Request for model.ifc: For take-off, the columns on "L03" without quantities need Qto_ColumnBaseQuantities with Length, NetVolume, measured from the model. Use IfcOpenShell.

First a look at what the model holds.

```python
import ifcopenshell
import ifcopenshell.util.element
import ifcopenshell.util.unit

model = ifcopenshell.open("model.ifc")
print(model.schema)
for unit_type in ("LENGTHUNIT", "AREAUNIT", "VOLUMEUNIT"):
    print(unit_type, ifcopenshell.util.unit.calculate_unit_scale(model, unit_type))
storey = next(s for s in model.by_type("IfcBuildingStorey") if s.Name == "L03")
columns = [e for e in ifcopenshell.util.element.get_decomposition(storey) if e.is_a("IfcColumn")]
for e in sorted(columns, key=lambda e: e.id()):
    print(e.id(), e.is_a(), e.Name, list(ifcopenshell.util.element.get_psets(e, qtos_only=True)), sep=" | ")
```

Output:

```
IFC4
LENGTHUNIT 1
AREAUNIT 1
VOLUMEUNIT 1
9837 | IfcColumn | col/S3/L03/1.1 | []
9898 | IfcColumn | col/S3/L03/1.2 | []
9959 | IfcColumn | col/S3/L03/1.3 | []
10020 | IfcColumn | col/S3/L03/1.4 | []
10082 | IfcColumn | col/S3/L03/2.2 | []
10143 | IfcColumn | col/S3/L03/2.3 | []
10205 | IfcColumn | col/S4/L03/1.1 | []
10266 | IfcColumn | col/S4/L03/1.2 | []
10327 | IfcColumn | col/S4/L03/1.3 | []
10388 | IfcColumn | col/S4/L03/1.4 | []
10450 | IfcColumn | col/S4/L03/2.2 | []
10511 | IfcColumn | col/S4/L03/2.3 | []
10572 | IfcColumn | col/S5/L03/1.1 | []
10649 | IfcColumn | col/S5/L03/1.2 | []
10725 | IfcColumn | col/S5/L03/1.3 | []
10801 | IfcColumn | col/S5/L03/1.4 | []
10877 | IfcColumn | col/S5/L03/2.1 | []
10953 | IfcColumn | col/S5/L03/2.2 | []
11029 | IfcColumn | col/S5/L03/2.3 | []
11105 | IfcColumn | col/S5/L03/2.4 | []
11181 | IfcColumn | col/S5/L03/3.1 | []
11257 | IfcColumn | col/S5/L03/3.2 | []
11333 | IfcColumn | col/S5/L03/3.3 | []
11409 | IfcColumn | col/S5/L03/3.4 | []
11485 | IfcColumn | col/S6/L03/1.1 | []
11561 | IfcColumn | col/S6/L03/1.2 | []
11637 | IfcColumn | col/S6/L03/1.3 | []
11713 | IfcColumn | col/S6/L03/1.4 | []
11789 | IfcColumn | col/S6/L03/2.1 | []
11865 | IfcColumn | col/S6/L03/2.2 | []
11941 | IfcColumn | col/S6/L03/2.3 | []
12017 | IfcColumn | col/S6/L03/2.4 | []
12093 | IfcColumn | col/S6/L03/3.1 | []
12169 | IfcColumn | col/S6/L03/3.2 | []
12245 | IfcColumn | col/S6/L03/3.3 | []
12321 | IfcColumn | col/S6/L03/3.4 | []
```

```python
import ifcopenshell
import ifcopenshell.api.pset
import ifcopenshell.geom
import ifcopenshell.util.element
import ifcopenshell.util.shape
import ifcopenshell.util.unit

model = ifcopenshell.open("model.ifc")
unit_scale = ifcopenshell.util.unit.calculate_unit_scale(model)
volume_scale = ifcopenshell.util.unit.calculate_unit_scale(model, "VOLUMEUNIT")
settings = ifcopenshell.geom.settings()

storey = next(s for s in model.by_type("IfcBuildingStorey") if s.Name == "L03")
columns = [e for e in ifcopenshell.util.element.get_decomposition(storey) if e.is_a("IfcColumn")]

for e in sorted(columns, key=lambda e: e.id()):
    if ifcopenshell.util.element.get_psets(e, qtos_only=True, should_inherit=False):
        continue
    # Geometry comes back in metres, in the element's own axes.
    shape = ifcopenshell.geom.create_shape(settings, e)
    values = {
        "Length": ifcopenshell.util.shape.get_z(shape.geometry) / unit_scale,
        "NetVolume": ifcopenshell.util.shape.get_volume(shape.geometry) / volume_scale,
    }
    qto = ifcopenshell.api.pset.add_qto(model, product=e, name="Qto_ColumnBaseQuantities")
    ifcopenshell.api.pset.edit_qto(model, qto=qto, properties=values)
    print(e.id(), {k: round(v, 3) for k, v in values.items()})

model.write("model_updated.ifc")
```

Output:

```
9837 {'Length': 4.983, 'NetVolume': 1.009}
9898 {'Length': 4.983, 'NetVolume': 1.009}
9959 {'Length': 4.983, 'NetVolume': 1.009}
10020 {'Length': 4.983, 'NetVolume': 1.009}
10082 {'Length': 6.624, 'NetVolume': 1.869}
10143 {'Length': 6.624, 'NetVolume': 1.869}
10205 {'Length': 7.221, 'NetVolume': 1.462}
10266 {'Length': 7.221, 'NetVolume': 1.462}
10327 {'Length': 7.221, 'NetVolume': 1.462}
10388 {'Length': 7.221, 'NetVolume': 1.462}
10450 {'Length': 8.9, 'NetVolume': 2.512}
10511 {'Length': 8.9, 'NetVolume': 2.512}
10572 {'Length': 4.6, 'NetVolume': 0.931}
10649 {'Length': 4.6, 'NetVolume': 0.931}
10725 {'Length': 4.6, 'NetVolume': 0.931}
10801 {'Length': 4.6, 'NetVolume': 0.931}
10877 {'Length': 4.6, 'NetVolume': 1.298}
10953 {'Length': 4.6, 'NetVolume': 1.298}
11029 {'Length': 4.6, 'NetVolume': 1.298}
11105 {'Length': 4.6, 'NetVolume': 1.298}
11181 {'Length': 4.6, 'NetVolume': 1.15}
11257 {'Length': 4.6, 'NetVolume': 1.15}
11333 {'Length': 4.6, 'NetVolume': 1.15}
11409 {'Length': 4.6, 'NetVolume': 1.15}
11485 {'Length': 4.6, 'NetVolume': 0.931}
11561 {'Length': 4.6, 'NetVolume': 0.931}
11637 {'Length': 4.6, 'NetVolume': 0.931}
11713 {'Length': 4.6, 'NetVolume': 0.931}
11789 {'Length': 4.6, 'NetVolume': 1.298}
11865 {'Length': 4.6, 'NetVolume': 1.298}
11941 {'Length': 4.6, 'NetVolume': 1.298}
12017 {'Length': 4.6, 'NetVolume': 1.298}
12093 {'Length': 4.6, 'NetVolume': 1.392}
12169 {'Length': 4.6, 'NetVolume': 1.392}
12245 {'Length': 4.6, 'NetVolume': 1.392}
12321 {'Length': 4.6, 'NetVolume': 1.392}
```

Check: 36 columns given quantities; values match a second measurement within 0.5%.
